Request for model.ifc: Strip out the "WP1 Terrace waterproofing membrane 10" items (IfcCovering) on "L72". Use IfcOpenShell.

First a look at what the model holds.

```python
import ifcopenshell
import ifcopenshell.util.element

model = ifcopenshell.open("model.ifc")
print(model.schema)
storey = next(s for s in model.by_type("IfcBuildingStorey") if s.Name == "L72")
coverings = [e for e in ifcopenshell.util.element.get_decomposition(storey) if e.is_a("IfcCovering")]
seen = {}
for e in coverings:
    element_type = ifcopenshell.util.element.get_type(e)
    name = element_type.Name if element_type not in (None, e) else None
    seen[name] = seen.get(name, 0) + 1
for name, count in sorted(seen.items(), key=str):
    print(count, "x", name)
```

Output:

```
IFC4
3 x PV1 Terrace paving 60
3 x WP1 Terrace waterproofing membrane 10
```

```python
import ifcopenshell
import ifcopenshell.api.root
import ifcopenshell.util.element

model = ifcopenshell.open("model.ifc")

storey = next(s for s in model.by_type("IfcBuildingStorey") if s.Name == "L72")
coverings = [e for e in ifcopenshell.util.element.get_decomposition(storey) if e.is_a("IfcCovering")]
targets = [e for e in coverings if (t := ifcopenshell.util.element.get_type(e)) not in (None, e) and t.Name == "WP1 Terrace waterproofing membrane 10"]

for e in targets:
    ifcopenshell.api.root.remove_product(model, product=e)
print(len(targets), "removed")

model.write("model_v2.ifc")
```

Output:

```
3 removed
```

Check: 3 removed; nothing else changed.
